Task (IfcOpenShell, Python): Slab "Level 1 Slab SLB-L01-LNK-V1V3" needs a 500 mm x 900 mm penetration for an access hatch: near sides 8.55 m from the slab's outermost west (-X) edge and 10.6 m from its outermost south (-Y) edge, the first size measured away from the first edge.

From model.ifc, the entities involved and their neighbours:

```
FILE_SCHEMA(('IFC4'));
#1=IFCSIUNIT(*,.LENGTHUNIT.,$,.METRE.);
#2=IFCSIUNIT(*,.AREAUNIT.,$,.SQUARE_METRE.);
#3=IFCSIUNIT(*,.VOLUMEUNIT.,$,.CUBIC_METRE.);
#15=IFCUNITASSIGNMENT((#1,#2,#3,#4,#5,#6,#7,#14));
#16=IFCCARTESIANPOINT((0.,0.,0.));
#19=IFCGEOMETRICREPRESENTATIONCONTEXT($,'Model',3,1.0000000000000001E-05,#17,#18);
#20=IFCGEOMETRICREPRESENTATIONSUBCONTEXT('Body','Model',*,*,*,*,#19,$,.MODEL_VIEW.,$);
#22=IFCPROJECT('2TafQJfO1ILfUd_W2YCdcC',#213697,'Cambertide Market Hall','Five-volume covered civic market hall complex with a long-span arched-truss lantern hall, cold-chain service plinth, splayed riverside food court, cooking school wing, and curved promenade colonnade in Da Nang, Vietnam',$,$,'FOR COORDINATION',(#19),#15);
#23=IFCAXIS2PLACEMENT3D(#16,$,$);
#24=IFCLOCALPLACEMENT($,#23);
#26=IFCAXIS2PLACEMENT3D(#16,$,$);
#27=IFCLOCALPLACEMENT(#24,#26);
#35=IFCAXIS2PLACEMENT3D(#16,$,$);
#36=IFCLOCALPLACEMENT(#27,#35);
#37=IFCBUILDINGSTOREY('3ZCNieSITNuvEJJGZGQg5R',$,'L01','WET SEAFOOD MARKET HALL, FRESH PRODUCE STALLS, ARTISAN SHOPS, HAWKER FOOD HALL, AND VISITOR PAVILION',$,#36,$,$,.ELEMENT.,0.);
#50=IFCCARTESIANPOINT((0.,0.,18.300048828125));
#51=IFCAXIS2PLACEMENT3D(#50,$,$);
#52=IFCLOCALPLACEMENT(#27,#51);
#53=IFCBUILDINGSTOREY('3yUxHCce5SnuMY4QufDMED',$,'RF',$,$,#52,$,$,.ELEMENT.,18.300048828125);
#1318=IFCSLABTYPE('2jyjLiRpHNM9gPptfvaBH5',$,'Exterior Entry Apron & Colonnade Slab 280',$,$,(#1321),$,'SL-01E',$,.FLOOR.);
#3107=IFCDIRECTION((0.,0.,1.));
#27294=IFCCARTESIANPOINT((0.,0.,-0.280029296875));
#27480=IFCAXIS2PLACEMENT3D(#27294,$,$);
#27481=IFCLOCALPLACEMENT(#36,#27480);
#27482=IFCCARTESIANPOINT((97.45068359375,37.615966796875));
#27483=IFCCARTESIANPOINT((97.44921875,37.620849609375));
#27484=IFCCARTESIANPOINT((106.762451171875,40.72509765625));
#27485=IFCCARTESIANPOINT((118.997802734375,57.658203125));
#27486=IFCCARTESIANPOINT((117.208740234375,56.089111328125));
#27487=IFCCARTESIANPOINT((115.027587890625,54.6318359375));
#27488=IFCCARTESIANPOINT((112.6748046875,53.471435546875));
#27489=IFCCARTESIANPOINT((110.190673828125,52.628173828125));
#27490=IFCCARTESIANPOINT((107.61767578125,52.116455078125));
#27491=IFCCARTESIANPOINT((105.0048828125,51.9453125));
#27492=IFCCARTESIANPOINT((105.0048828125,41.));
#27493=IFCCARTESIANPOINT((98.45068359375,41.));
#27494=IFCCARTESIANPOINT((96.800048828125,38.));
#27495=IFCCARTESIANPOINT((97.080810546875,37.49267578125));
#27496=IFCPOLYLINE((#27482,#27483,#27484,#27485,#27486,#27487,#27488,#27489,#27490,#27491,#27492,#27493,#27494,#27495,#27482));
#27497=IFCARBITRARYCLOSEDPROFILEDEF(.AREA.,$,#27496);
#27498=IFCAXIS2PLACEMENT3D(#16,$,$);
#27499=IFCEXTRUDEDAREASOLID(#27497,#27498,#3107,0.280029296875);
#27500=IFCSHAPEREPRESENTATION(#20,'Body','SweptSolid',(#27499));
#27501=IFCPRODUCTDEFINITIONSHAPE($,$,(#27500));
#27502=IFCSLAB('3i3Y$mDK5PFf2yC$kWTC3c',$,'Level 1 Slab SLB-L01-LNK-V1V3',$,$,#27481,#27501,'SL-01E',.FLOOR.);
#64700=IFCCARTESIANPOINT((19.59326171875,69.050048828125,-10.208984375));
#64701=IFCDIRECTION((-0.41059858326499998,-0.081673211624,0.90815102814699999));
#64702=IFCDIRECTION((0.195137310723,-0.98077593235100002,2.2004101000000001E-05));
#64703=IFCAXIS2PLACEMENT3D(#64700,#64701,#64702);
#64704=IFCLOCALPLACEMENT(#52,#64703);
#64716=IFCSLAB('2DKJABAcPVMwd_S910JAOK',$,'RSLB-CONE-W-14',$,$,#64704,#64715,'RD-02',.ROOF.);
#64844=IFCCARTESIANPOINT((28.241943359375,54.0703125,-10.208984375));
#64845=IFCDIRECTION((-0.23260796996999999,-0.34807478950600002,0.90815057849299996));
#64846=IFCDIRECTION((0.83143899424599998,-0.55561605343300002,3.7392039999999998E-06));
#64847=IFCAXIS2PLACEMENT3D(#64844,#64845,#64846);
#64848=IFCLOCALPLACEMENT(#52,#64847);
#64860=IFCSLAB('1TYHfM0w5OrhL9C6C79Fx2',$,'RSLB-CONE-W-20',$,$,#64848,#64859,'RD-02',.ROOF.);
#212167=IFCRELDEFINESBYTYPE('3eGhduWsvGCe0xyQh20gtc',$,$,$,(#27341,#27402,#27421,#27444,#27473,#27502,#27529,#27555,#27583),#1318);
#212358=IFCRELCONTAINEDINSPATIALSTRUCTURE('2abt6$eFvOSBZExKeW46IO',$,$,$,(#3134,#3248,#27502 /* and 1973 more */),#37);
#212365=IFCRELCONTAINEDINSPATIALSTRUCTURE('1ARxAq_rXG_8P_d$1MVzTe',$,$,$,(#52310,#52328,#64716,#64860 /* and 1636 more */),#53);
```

```python
import numpy as np
import ifcopenshell
import ifcopenshell.api.feature
import ifcopenshell.api.geometry
import ifcopenshell.api.root
import ifcopenshell.geom
import ifcopenshell.util.placement
import ifcopenshell.util.representation
import ifcopenshell.util.shape
import ifcopenshell.util.unit

model = ifcopenshell.open("model.ifc")
unit_scale = ifcopenshell.util.unit.calculate_unit_scale(model)
settings = ifcopenshell.geom.settings()


def volume(element):
    """Net volume in cubic metres, openings subtracted."""
    shape = ifcopenshell.geom.create_shape(settings, element)
    return ifcopenshell.util.shape.get_volume(shape.geometry)


slab = model.by_guid("3i3Y$mDK5PFf2yC$kWTC3c")
before = volume(slab)

# Extent in the slab's own axes, in metres. The edges named are its -X and -Y sides.
slab_shape = ifcopenshell.geom.create_shape(settings, slab)
vertices = ifcopenshell.util.shape.get_vertices(slab_shape.geometry)
x_min, y_min, bottom = vertices.min(axis=0)
top = vertices[:, 2].max()

opening = ifcopenshell.api.root.create_entity(model, ifc_class="IfcOpeningElement", name="Access hatch opening", predefined_type="OPENING")
context = ifcopenshell.util.representation.get_context(model, "Model", "Body", "MODEL_VIEW")
width, depth = 0.5, 0.9
outline = [(0.0, 0.0), (width, 0.0), (width, depth), (0.0, depth), (0.0, 0.0)]
# Overshoot both faces by 50 mm so the cut is clean.
shape = ifcopenshell.api.geometry.add_slab_representation(
    model, context=context, depth=top - bottom + 0.1, polyline=outline
)
ifcopenshell.api.geometry.assign_representation(model, product=opening, representation=shape)

matrix = ifcopenshell.util.placement.get_local_placement(slab.ObjectPlacement)
matrix[:, 3] = matrix @ np.append(np.array([x_min + 8.55, y_min + 10.6, bottom - 0.05]) / unit_scale, 1.0)
ifcopenshell.api.geometry.edit_object_placement(model, product=opening, matrix=matrix, is_si=False)
ifcopenshell.api.feature.add_feature(model, feature=opening, element=slab)

after = volume(slab)

print(f"slab volume {before:.3f} -> {after:.3f} m3")

model.write("model_updated.ifc")
```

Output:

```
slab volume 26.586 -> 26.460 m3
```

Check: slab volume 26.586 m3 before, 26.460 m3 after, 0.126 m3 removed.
